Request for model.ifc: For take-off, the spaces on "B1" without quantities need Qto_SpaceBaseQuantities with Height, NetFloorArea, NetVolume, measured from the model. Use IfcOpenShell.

First a look at what the model holds.

```python
import ifcopenshell
import ifcopenshell.util.element
import ifcopenshell.util.unit

model = ifcopenshell.open("model.ifc")
print(model.schema)
for unit_type in ("LENGTHUNIT", "AREAUNIT", "VOLUMEUNIT"):
    print(unit_type, ifcopenshell.util.unit.calculate_unit_scale(model, unit_type))
storey = next(s for s in model.by_type("IfcBuildingStorey") if s.Name == "B1")
spaces = [e for e in ifcopenshell.util.element.get_decomposition(storey) if e.is_a("IfcSpace")]
for e in sorted(spaces, key=lambda e: e.id()):
    print(e.id(), e.is_a(), e.Name, list(ifcopenshell.util.element.get_psets(e, qtos_only=True)), sep=" | ")
```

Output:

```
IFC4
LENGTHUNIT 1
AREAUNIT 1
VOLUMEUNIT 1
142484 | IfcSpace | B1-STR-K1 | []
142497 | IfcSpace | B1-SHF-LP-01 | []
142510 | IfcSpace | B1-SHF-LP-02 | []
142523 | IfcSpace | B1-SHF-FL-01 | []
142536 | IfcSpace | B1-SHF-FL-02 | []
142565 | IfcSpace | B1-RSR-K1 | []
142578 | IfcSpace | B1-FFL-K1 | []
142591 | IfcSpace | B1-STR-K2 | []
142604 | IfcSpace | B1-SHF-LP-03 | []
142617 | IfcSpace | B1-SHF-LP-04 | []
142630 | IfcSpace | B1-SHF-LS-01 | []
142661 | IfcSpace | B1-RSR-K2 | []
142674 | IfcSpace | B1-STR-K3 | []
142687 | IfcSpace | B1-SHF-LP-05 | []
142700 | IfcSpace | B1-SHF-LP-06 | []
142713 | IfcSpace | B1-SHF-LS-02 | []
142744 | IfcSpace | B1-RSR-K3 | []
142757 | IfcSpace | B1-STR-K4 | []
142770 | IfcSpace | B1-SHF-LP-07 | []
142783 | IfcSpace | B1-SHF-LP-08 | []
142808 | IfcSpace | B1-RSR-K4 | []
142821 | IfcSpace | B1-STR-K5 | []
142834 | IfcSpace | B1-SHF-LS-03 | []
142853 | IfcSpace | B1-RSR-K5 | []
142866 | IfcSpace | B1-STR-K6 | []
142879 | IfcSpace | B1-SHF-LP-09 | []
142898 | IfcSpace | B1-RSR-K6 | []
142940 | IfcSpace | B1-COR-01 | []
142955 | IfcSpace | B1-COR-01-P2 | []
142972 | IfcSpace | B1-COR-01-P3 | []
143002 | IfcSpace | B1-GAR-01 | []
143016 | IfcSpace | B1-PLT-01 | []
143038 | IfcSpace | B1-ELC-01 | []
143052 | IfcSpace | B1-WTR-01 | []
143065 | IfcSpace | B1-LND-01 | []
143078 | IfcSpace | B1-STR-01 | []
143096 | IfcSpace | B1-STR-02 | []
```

```python
import ifcopenshell
import ifcopenshell.api.pset
import ifcopenshell.geom
import ifcopenshell.util.element
import ifcopenshell.util.shape
import ifcopenshell.util.unit

model = ifcopenshell.open("model.ifc")
unit_scale = ifcopenshell.util.unit.calculate_unit_scale(model)
area_scale = ifcopenshell.util.unit.calculate_unit_scale(model, "AREAUNIT")
volume_scale = ifcopenshell.util.unit.calculate_unit_scale(model, "VOLUMEUNIT")
settings = ifcopenshell.geom.settings()

storey = next(s for s in model.by_type("IfcBuildingStorey") if s.Name == "B1")
spaces = [e for e in ifcopenshell.util.element.get_decomposition(storey) if e.is_a("IfcSpace")]

for e in sorted(spaces, key=lambda e: e.id()):
    if ifcopenshell.util.element.get_psets(e, qtos_only=True, should_inherit=False):
        continue
    # Geometry comes back in metres, in the element's own axes.
    shape = ifcopenshell.geom.create_shape(settings, e)
    values = {
        "Height": ifcopenshell.util.shape.get_z(shape.geometry) / unit_scale,
        "NetFloorArea": ifcopenshell.util.shape.get_footprint_area(shape.geometry) / area_scale,
        "NetVolume": ifcopenshell.util.shape.get_volume(shape.geometry) / volume_scale,
    }
    qto = ifcopenshell.api.pset.add_qto(model, product=e, name="Qto_SpaceBaseQuantities")
    ifcopenshell.api.pset.edit_qto(model, qto=qto, properties=values)
    print(e.id(), {k: round(v, 3) for k, v in values.items()})

model.write("model_edited.ifc")
```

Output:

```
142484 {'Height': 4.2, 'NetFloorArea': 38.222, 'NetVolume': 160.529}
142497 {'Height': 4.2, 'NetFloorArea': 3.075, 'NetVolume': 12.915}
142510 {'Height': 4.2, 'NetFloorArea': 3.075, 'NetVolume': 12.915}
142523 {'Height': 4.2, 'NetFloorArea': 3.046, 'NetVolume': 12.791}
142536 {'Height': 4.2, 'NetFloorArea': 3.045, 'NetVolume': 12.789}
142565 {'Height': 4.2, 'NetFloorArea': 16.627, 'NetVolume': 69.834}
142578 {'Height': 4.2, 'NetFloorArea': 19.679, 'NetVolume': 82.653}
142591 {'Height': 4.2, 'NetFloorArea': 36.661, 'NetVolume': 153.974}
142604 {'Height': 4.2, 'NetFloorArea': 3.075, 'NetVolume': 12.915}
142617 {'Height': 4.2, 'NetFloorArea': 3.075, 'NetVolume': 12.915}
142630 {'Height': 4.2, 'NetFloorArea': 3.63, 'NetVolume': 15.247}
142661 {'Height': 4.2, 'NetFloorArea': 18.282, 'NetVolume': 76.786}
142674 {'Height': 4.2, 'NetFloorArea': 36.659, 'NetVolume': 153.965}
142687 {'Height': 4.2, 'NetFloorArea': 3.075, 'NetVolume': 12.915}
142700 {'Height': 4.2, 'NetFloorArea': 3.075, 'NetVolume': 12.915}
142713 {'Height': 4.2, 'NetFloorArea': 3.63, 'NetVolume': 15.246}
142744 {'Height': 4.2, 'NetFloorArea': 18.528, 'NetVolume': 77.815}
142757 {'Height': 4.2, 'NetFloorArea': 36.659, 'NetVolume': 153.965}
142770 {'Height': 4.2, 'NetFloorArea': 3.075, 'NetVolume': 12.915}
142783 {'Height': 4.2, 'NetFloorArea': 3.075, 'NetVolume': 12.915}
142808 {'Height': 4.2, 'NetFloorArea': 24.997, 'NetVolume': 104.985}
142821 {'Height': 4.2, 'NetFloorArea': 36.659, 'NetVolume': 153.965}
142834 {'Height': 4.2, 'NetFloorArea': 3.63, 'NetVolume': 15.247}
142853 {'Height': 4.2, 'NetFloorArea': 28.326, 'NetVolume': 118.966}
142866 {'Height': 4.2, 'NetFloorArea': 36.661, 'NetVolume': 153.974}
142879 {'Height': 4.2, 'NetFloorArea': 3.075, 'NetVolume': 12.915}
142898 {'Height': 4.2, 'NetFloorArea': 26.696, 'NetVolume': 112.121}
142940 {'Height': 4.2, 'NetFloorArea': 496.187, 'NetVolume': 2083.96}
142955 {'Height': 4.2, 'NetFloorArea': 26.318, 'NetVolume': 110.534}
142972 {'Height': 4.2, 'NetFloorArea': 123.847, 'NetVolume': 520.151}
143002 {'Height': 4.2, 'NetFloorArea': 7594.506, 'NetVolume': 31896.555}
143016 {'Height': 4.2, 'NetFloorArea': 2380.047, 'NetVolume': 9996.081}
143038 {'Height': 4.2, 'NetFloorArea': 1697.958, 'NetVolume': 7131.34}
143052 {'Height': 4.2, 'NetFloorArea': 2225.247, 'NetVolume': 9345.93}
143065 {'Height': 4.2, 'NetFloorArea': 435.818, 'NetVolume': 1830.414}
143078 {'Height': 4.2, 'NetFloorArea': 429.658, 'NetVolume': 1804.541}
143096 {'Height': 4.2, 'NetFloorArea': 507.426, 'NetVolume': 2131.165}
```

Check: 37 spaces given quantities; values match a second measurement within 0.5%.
